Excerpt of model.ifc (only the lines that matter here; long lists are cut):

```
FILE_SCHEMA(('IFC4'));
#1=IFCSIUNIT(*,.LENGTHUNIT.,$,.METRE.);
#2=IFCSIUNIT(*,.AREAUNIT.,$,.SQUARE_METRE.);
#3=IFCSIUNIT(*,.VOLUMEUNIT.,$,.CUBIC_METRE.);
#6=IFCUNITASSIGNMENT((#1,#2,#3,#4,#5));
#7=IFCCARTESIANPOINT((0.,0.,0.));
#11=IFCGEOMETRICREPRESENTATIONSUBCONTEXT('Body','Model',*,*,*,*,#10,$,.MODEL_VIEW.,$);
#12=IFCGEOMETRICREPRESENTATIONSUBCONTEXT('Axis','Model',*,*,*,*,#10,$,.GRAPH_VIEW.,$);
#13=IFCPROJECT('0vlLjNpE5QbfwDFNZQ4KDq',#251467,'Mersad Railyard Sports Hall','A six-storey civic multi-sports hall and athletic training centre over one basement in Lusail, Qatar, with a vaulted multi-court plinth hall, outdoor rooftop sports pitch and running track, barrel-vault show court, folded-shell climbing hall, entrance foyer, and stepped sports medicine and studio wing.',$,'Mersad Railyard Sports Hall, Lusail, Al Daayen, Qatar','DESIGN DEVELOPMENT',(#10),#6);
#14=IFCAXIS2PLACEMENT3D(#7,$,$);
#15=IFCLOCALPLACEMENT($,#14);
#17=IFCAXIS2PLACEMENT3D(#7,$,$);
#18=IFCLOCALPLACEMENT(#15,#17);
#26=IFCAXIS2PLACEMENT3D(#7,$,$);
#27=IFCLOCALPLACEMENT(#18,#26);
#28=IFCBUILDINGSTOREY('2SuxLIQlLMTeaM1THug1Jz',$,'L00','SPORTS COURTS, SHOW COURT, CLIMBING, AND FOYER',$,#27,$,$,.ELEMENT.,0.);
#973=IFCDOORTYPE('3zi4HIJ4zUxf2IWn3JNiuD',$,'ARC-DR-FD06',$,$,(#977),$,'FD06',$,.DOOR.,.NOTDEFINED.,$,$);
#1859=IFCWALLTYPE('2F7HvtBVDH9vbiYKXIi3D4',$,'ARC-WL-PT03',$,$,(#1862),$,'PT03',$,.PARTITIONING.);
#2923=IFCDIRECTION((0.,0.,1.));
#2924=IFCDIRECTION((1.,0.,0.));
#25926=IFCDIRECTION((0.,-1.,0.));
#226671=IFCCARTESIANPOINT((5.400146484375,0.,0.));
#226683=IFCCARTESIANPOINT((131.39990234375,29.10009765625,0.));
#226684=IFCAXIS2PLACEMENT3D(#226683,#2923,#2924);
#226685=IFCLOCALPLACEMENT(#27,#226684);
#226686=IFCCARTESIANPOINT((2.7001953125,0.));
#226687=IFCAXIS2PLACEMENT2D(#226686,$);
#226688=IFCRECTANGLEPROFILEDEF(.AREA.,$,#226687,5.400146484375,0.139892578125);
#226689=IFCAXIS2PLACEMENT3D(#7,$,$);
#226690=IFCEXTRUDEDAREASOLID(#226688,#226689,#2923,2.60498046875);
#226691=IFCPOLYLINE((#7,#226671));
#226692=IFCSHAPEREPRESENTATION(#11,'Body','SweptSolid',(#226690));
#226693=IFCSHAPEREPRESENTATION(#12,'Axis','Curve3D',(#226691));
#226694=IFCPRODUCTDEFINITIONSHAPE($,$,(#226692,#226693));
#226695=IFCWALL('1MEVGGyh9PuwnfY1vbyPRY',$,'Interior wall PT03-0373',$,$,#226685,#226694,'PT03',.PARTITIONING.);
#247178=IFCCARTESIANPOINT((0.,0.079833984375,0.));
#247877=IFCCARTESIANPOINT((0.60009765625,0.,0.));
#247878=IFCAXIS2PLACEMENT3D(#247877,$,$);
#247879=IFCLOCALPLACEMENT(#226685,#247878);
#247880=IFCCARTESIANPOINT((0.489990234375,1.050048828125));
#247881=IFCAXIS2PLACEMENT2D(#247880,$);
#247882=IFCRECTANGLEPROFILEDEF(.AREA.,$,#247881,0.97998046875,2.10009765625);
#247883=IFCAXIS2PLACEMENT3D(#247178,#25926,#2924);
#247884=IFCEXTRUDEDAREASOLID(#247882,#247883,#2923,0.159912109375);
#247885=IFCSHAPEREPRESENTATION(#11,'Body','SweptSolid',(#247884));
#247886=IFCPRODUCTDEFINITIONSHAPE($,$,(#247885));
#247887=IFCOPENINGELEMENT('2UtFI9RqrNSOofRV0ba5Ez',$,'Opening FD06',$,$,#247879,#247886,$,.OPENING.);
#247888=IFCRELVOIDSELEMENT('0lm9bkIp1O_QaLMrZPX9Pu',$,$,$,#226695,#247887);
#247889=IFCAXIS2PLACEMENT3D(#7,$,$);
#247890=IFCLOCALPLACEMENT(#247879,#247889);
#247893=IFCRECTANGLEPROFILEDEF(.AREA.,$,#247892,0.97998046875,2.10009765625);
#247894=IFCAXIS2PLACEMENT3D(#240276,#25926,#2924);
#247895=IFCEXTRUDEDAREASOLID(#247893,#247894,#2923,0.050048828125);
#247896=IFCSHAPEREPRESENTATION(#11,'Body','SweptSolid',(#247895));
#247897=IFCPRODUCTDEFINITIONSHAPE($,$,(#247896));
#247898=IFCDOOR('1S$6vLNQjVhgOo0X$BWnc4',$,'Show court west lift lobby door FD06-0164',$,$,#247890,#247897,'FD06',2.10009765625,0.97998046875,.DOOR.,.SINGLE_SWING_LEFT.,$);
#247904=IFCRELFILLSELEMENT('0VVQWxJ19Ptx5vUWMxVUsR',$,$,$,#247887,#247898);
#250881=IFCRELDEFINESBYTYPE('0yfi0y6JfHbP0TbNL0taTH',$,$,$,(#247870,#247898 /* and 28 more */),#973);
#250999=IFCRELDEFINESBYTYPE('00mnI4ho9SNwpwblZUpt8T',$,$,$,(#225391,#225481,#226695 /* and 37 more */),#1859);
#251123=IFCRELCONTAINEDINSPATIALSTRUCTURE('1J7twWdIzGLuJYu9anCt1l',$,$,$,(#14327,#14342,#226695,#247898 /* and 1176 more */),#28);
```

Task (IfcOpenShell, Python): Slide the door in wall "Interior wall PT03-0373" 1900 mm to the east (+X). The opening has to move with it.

```python
import ifcopenshell
import ifcopenshell.api.geometry
import ifcopenshell.util.placement
import ifcopenshell.util.unit

model = ifcopenshell.open("model.ifc")
unit_scale = ifcopenshell.util.unit.calculate_unit_scale(model)

door = model.by_guid("1S$6vLNQjVhgOo0X$BWnc4")
opening = door.FillsVoids[0].RelatingOpeningElement
wall = opening.VoidsElements[0].RelatingBuildingElement

wall_matrix = ifcopenshell.util.placement.get_local_placement(wall.ObjectPlacement)
shift = wall_matrix[:3, 0] * 1.9 / unit_scale
before = ifcopenshell.util.placement.get_local_placement(door.ObjectPlacement)[:3, 3].copy()

# The door is placed relative to its opening, so it follows when the opening moves.
matrix = ifcopenshell.util.placement.get_local_placement(opening.ObjectPlacement)
matrix[:3, 3] += shift
ifcopenshell.api.geometry.edit_object_placement(
    model, product=opening, matrix=matrix, is_si=False, should_transform_children=True
)

after = ifcopenshell.util.placement.get_local_placement(door.ObjectPlacement)[:3, 3]
print("door moved by", (after - before).round(3) + 0.0)

model.write("model-out.ifc")
```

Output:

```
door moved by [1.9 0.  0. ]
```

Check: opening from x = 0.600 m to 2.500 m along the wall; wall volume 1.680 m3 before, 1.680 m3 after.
